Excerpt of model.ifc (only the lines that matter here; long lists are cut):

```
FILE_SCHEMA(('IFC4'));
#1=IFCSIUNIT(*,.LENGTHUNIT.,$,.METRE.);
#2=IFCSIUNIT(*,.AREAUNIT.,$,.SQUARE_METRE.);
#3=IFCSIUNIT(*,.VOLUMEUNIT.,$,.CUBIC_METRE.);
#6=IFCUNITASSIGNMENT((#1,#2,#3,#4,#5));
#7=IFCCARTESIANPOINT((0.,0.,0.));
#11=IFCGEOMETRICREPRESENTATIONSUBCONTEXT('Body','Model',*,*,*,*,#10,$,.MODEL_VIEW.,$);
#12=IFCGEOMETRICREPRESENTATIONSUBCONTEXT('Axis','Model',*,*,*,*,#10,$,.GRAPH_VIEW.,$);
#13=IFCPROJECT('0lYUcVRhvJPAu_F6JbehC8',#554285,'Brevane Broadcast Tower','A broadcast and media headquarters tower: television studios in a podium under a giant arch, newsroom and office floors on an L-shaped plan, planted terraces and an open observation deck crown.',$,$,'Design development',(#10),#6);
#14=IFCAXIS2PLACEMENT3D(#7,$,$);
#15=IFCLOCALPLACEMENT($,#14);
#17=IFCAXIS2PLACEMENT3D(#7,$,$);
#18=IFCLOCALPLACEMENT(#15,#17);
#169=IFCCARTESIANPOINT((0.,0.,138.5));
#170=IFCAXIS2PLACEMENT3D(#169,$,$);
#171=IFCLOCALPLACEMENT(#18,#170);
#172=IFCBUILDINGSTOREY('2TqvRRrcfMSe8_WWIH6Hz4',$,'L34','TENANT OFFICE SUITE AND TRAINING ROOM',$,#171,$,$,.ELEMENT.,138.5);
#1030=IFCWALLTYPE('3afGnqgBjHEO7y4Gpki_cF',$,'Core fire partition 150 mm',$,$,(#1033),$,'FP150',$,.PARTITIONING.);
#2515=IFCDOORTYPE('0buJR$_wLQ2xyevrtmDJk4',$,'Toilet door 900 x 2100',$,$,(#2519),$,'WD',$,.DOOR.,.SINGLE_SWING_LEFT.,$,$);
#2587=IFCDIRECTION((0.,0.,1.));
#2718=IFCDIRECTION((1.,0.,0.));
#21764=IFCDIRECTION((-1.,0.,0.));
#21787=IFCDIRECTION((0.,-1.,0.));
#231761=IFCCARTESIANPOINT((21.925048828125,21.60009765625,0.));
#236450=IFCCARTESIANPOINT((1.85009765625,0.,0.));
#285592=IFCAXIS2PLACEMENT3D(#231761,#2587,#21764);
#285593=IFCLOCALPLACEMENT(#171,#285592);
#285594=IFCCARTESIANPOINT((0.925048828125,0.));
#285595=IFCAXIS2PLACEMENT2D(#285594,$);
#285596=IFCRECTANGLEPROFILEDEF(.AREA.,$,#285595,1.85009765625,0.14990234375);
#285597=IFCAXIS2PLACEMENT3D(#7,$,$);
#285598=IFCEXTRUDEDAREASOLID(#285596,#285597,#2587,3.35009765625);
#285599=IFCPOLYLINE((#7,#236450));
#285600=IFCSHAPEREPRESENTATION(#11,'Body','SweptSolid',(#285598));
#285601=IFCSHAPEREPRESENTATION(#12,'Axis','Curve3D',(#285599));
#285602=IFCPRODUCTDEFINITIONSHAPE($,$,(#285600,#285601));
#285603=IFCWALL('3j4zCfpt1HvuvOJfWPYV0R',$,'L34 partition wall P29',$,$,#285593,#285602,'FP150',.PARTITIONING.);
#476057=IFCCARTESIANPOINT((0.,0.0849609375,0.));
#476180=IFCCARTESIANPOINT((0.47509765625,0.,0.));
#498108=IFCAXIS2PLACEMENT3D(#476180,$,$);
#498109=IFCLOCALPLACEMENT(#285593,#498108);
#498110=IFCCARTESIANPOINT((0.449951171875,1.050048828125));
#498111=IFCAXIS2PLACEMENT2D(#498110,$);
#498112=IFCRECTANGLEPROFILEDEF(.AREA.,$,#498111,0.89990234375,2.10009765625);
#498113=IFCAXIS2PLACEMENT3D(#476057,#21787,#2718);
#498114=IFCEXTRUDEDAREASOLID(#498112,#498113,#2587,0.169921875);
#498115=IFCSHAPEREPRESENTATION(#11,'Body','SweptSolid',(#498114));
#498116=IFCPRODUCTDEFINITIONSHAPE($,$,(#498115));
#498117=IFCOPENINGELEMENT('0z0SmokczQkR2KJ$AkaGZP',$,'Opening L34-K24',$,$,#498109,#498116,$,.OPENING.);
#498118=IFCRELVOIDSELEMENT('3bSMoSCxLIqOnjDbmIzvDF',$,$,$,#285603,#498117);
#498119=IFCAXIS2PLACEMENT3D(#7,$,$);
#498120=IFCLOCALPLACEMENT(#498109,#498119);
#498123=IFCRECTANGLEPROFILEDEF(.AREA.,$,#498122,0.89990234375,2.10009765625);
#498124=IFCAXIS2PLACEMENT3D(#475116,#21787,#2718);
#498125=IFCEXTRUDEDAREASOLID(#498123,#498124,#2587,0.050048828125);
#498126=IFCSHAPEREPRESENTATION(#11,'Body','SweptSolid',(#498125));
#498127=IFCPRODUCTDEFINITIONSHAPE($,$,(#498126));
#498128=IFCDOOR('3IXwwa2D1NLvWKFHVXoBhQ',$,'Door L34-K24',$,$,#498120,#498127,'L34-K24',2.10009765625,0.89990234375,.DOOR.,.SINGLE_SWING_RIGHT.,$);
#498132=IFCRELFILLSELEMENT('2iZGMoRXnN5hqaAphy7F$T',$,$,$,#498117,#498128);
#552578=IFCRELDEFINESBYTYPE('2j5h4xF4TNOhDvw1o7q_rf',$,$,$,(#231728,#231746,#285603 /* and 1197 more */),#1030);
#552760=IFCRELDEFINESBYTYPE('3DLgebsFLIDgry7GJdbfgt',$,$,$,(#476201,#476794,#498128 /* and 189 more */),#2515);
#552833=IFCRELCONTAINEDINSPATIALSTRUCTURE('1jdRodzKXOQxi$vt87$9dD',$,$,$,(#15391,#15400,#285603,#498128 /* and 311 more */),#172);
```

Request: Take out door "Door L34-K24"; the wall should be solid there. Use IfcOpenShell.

```python
import ifcopenshell
import ifcopenshell.api.feature
import ifcopenshell.api.root
import ifcopenshell.geom
import ifcopenshell.util.shape

model = ifcopenshell.open("model.ifc")
settings = ifcopenshell.geom.settings()


def volume(element):
    """Net volume in cubic metres, openings subtracted."""
    shape = ifcopenshell.geom.create_shape(settings, element)
    return ifcopenshell.util.shape.get_volume(shape.geometry)


door = model.by_guid("3IXwwa2D1NLvWKFHVXoBhQ")
opening = door.FillsVoids[0].RelatingOpeningElement
wall = opening.VoidsElements[0].RelatingBuildingElement
before = volume(wall)

ifcopenshell.api.root.remove_product(model, product=door)
ifcopenshell.api.feature.remove_feature(model, feature=opening)

after = volume(wall)

print(f"wall volume {before:.3f} -> {after:.3f} m3")

model.write("model_v2.ifc")
```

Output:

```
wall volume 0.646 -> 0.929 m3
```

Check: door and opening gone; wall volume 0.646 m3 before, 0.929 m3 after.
